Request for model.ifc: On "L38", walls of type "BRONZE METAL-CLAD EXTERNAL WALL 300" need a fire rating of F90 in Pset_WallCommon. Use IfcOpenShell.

First a look at what the model holds.

```python
import ifcopenshell
import ifcopenshell.util.element

model = ifcopenshell.open("model.ifc")
print(model.schema)
storey = next(s for s in model.by_type("IfcBuildingStorey") if s.Name == "L38")
walls = [e for e in ifcopenshell.util.element.get_decomposition(storey) if e.is_a("IfcWall")]
seen = {}
for e in walls:
    element_type = ifcopenshell.util.element.get_type(e)
    key = (element_type.Name if element_type != e and element_type else None, ifcopenshell.util.element.get_pset(e, "Pset_WallCommon", "FireRating"))
    seen[key] = seen.get(key, 0) + 1
for (name, value), count in sorted(seen.items(), key=str):
    print(count, "x", name, "|", value)
```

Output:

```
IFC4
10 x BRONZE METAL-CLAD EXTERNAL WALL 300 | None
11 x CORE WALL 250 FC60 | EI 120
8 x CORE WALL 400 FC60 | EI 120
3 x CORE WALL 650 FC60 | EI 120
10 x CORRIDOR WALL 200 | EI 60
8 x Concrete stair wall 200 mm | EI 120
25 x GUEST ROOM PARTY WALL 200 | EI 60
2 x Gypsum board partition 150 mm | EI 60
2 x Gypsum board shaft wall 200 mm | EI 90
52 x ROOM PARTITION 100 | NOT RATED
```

```python
import ifcopenshell
import ifcopenshell.api.pset
import ifcopenshell.util.element

model = ifcopenshell.open("model.ifc")

storey = next(s for s in model.by_type("IfcBuildingStorey") if s.Name == "L38")
walls = [e for e in ifcopenshell.util.element.get_decomposition(storey) if e.is_a("IfcWall")]

count = 0
for e in walls:
    element_type = ifcopenshell.util.element.get_type(e)
    if element_type in (None, e) or element_type.Name != "BRONZE METAL-CLAD EXTERNAL WALL 300":
        continue
    found = ifcopenshell.util.element.get_pset(e, "Pset_WallCommon", should_inherit=False)
    if found:
        pset = model.by_id(found["id"])
        if len(ifcopenshell.util.element.get_elements_by_pset(pset)) > 1:
            pset = ifcopenshell.api.pset.unshare_pset(model, products=[e], pset=pset)[0]
    else:
        pset = ifcopenshell.api.pset.add_pset(model, product=e, name="Pset_WallCommon")
    ifcopenshell.api.pset.edit_pset(model, pset=pset, properties={"FireRating": "F90"})
    count += 1

print(count, "walls updated")

model.write("model_updated.ifc")
```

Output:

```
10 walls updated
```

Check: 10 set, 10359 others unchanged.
